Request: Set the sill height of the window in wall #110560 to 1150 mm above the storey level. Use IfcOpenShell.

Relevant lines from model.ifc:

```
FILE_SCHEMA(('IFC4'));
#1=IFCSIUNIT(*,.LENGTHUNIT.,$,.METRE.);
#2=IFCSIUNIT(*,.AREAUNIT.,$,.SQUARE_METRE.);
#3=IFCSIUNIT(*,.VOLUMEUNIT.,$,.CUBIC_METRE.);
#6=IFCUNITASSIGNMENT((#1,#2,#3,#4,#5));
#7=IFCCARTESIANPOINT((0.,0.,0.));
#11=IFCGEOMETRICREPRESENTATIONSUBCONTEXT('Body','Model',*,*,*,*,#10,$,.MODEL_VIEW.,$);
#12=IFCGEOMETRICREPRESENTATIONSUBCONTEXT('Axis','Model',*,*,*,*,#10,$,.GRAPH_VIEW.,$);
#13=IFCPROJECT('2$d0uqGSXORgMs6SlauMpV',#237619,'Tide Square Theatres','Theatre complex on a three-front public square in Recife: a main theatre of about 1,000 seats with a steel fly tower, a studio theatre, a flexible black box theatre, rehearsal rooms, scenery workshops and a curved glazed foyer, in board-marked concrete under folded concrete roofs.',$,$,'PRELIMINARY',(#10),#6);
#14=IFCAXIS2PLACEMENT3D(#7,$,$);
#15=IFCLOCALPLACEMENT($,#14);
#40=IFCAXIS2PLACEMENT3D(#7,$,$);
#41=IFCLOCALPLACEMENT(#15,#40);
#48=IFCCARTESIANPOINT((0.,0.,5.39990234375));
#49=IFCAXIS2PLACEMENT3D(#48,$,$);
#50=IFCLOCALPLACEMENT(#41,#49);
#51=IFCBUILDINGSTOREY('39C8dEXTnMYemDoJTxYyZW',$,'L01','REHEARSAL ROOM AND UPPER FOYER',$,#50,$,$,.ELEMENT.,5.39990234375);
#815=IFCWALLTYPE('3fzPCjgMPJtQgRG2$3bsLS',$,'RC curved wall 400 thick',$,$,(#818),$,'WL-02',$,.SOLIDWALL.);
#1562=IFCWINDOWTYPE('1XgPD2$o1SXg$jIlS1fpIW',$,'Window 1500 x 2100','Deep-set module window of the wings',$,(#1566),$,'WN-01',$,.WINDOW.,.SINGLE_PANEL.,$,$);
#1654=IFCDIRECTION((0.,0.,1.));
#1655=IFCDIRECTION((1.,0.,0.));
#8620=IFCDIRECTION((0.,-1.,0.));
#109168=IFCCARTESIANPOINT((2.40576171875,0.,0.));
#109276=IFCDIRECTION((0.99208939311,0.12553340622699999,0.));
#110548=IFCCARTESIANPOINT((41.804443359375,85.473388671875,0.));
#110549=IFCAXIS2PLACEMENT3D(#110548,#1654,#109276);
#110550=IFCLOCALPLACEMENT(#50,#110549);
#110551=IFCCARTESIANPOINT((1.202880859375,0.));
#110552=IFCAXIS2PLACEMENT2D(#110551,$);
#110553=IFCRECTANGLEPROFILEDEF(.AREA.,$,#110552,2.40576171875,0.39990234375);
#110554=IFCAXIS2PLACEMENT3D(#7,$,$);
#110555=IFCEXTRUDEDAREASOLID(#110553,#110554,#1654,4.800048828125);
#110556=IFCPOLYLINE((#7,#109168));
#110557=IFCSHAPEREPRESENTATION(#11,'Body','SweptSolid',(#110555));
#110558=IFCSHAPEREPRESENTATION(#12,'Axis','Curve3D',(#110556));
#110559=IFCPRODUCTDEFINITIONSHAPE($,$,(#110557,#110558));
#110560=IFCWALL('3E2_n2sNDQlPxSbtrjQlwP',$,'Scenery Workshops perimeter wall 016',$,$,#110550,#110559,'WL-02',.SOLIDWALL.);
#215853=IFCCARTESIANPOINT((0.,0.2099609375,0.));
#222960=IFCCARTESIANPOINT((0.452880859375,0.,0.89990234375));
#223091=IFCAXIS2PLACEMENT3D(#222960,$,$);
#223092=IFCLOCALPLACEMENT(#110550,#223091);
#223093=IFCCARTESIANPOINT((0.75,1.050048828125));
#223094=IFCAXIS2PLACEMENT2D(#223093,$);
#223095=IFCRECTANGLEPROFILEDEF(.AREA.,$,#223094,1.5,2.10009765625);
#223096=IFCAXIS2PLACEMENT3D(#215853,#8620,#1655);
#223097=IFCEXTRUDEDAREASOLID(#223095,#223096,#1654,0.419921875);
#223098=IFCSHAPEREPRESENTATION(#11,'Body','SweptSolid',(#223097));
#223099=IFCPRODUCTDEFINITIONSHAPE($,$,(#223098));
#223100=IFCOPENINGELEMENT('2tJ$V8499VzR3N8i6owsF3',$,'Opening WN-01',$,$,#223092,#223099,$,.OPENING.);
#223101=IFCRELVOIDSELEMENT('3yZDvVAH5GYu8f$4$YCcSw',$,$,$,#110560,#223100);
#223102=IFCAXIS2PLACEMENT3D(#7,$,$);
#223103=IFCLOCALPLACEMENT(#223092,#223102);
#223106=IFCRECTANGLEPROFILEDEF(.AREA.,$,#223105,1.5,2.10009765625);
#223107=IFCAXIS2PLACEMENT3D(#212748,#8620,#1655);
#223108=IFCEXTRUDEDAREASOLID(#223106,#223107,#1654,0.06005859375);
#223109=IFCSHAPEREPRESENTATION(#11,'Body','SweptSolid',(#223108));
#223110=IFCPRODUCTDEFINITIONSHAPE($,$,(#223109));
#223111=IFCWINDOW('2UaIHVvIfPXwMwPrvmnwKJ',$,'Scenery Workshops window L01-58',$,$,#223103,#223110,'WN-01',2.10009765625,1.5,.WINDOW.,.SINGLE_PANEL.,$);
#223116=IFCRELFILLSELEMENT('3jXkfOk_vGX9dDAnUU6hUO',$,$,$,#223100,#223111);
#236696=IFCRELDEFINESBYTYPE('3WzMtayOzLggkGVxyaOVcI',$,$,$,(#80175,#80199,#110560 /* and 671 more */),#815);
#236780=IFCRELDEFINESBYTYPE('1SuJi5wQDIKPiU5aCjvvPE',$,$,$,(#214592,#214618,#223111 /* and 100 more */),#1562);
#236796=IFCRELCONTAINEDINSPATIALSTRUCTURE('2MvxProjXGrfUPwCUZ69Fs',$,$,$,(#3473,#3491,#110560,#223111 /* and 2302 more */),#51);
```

```python
import numpy as np
import ifcopenshell
import ifcopenshell.api.geometry
import ifcopenshell.geom
import ifcopenshell.util.element
import ifcopenshell.util.placement
import ifcopenshell.util.shape
import ifcopenshell.util.unit

model = ifcopenshell.open("model.ifc")
unit_scale = ifcopenshell.util.unit.calculate_unit_scale(model)

window = model.by_guid("2UaIHVvIfPXwMwPrvmnwKJ")
opening = window.FillsVoids[0].RelatingOpeningElement
storey = ifcopenshell.util.element.get_container(window, ifc_class="IfcBuildingStorey")
level = ifcopenshell.util.placement.get_local_placement(storey.ObjectPlacement)[2, 3]

# The opening's origin need not be at the sill, so measure its lowest point.
shape = ifcopenshell.geom.create_shape(ifcopenshell.geom.settings(), opening)
bottom = ifcopenshell.util.shape.get_shape_bottom_elevation(shape, shape.geometry) / unit_scale
dz = level + 1.15 / unit_scale - bottom

shift = np.array([0.0, 0.0, dz])
# The window is placed relative to its opening, so it follows when the opening moves.
matrix = ifcopenshell.util.placement.get_local_placement(opening.ObjectPlacement)
matrix[:3, 3] += shift
ifcopenshell.api.geometry.edit_object_placement(
    model, product=opening, matrix=matrix, is_si=False, should_transform_children=True
)

print(f"moved by {dz * unit_scale:+.3f} m")

model.write("model_edited.ifc")
```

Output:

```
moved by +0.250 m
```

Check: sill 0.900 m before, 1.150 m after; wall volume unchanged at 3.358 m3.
